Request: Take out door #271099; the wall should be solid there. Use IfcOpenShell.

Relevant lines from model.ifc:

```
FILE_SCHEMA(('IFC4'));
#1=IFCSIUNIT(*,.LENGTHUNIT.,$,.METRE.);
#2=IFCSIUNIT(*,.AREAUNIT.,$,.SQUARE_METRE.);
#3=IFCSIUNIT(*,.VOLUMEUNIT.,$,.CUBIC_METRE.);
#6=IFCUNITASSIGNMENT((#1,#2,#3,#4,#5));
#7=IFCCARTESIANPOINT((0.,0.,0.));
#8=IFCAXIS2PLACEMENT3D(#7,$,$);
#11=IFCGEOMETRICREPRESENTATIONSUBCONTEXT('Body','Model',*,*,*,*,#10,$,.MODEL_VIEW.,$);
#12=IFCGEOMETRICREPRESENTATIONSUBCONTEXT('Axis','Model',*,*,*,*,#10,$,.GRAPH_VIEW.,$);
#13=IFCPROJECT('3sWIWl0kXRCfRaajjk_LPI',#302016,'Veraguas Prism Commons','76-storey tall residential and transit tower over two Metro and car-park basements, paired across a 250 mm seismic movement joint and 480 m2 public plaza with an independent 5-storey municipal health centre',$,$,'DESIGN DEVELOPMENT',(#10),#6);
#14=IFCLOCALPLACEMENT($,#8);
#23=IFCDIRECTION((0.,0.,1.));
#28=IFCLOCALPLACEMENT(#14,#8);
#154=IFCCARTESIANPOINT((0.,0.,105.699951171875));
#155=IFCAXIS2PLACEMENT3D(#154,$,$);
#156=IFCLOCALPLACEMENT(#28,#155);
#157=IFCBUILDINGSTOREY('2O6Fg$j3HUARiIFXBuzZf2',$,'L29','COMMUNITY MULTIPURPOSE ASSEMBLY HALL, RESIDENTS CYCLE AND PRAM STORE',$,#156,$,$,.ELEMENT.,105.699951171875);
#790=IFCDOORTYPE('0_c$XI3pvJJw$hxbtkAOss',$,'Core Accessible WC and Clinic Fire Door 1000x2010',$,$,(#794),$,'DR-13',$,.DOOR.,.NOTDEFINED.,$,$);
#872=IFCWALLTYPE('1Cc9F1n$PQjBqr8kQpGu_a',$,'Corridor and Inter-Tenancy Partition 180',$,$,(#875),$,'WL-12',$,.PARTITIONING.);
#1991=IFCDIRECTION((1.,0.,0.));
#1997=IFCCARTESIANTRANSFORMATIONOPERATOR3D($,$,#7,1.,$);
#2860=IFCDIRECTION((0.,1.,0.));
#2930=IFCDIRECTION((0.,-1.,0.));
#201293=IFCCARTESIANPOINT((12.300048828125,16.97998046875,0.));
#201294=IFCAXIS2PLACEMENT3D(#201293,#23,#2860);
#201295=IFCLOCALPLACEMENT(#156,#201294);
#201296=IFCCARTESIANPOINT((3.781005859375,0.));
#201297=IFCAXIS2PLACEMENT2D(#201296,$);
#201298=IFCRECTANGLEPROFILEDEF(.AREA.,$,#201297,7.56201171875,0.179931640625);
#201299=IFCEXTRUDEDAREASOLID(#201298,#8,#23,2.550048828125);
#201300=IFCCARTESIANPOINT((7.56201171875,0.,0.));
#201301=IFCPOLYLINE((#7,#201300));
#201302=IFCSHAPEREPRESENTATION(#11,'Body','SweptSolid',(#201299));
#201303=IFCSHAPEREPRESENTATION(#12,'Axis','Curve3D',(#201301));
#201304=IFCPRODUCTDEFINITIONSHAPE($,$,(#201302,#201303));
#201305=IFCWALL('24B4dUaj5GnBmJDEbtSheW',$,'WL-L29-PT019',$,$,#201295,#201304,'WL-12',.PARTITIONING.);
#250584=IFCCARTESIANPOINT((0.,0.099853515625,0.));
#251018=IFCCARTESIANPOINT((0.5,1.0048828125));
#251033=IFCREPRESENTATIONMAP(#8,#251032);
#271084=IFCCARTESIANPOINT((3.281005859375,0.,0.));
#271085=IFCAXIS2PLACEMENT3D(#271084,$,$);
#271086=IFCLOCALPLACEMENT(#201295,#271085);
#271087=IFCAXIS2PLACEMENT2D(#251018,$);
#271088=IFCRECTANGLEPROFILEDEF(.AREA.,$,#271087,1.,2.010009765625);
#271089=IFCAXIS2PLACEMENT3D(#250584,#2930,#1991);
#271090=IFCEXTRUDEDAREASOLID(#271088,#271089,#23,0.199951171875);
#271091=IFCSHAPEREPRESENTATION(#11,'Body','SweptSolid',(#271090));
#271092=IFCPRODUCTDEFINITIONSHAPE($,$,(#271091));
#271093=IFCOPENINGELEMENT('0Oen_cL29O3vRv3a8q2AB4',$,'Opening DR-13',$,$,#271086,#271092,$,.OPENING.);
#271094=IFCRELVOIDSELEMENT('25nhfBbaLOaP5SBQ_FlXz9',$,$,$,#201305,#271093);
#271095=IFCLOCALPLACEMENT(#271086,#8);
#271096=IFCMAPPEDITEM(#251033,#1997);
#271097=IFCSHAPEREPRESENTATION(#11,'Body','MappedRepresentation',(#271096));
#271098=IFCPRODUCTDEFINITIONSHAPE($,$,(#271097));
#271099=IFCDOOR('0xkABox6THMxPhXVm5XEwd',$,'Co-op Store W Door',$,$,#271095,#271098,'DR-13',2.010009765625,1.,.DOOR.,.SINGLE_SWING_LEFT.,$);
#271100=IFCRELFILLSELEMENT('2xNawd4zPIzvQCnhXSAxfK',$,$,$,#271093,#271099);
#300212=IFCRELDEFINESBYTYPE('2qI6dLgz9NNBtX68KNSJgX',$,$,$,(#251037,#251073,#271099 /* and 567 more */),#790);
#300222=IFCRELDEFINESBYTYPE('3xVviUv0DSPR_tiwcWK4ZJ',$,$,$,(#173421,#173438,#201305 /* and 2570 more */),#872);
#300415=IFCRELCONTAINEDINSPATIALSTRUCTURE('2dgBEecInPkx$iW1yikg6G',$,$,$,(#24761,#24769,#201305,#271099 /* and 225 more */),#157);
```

```python
import ifcopenshell
import ifcopenshell.api.feature
import ifcopenshell.api.root
import ifcopenshell.geom
import ifcopenshell.util.shape

model = ifcopenshell.open("model.ifc")
settings = ifcopenshell.geom.settings()


def volume(element):
    """Net volume in cubic metres, openings subtracted."""
    shape = ifcopenshell.geom.create_shape(settings, element)
    return ifcopenshell.util.shape.get_volume(shape.geometry)


door = model.by_id(271099)
opening = door.FillsVoids[0].RelatingOpeningElement
wall = opening.VoidsElements[0].RelatingBuildingElement
before = volume(wall)

ifcopenshell.api.root.remove_product(model, product=door)
ifcopenshell.api.feature.remove_feature(model, feature=opening)

after = volume(wall)

print(f"wall volume {before:.3f} -> {after:.3f} m3")

model.write("model_rev.ifc")
```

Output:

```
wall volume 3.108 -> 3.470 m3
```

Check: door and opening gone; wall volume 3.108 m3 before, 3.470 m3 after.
